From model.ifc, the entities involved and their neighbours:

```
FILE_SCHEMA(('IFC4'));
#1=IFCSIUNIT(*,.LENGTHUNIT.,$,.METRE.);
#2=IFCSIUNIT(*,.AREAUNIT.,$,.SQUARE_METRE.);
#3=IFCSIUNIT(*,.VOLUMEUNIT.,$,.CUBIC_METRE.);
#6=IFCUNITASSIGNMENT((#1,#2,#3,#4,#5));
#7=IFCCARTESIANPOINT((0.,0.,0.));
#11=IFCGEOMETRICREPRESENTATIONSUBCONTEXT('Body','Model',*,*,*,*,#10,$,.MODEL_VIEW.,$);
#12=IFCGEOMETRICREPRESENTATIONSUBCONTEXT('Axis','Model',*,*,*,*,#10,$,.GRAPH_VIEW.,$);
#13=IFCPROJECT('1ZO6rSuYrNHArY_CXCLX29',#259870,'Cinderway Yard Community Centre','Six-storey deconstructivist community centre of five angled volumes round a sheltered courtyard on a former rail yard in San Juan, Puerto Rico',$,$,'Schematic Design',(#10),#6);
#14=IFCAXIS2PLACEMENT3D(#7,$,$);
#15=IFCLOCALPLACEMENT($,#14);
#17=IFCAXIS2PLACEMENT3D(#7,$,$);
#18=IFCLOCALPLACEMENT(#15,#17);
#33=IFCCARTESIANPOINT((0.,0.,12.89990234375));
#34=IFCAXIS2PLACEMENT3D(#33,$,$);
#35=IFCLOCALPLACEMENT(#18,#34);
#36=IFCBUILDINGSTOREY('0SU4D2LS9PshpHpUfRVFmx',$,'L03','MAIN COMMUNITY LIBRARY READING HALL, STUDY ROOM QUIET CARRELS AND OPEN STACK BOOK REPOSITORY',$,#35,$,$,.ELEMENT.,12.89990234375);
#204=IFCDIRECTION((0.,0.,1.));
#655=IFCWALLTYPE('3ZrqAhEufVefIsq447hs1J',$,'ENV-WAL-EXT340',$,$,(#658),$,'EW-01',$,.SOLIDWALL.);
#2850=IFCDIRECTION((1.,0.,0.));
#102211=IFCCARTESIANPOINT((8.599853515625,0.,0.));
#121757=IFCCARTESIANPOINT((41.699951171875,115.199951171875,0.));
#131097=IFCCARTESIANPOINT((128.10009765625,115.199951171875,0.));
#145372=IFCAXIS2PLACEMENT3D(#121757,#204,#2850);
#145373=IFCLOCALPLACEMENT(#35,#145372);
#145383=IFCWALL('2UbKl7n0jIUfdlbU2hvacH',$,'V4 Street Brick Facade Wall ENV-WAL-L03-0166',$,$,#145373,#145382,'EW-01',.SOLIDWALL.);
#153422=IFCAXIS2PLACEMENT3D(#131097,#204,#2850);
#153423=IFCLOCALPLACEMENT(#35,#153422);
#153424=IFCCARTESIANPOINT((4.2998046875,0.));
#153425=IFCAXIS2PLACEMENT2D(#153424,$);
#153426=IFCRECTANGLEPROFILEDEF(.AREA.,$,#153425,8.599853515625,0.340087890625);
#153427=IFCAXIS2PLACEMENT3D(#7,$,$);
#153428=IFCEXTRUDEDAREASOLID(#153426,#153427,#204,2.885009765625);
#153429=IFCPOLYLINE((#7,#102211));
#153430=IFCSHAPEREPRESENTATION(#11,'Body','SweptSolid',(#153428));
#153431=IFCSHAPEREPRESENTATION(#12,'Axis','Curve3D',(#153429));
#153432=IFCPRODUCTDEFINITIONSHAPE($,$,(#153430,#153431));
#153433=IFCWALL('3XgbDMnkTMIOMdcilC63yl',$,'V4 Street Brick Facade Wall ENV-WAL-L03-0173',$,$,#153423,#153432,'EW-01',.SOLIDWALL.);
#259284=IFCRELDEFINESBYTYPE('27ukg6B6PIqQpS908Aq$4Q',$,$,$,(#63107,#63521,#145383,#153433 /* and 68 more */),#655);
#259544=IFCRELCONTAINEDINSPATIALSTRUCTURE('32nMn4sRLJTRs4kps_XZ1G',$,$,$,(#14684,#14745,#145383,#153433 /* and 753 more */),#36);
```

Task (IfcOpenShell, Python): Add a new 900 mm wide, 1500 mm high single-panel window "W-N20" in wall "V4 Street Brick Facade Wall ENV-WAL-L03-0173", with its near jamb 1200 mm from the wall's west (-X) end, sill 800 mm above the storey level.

```python
import numpy as np
import ifcopenshell
import ifcopenshell.api.feature
import ifcopenshell.api.geometry
import ifcopenshell.api.root
import ifcopenshell.api.spatial
import ifcopenshell.geom
import ifcopenshell.util.element
import ifcopenshell.util.placement
import ifcopenshell.util.representation
import ifcopenshell.util.shape
import ifcopenshell.util.unit

model = ifcopenshell.open("model.ifc")
unit_scale = ifcopenshell.util.unit.calculate_unit_scale(model)
settings = ifcopenshell.geom.settings()


def volume(element):
    """Net volume in cubic metres, openings subtracted."""
    shape = ifcopenshell.geom.create_shape(settings, element)
    return ifcopenshell.util.shape.get_volume(shape.geometry)


wall = model.by_guid("3XgbDMnkTMIOMdcilC63yl")
storey = ifcopenshell.util.element.get_container(wall, ifc_class="IfcBuildingStorey")
context = ifcopenshell.util.representation.get_context(model, "Model", "Body", "MODEL_VIEW")
before = volume(wall)

width, height, from_end, sill = 0.9, 1.5, 1.2, 0.8  # metres

# The wall runs along its own X axis, and the end named is its -X end.
wall_shape = ifcopenshell.geom.create_shape(settings, wall)
x, y, z = ifcopenshell.util.shape.get_vertices(wall_shape.geometry).T
start = x.min() + from_end
face, thickness = float(y.min()), float(y.max() - y.min())
wall_matrix = ifcopenshell.util.placement.get_local_placement(wall.ObjectPlacement)
level = ifcopenshell.util.placement.get_local_placement(storey.ObjectPlacement)[2, 3]


def in_wall(x, y):
    """Placement at x, y metres in the wall's axes, at sill height."""
    matrix = wall_matrix.copy()
    matrix[:, 3] = wall_matrix @ np.array([x / unit_scale, y / unit_scale, 0.0, 1.0])
    matrix[2, 3] = level + sill / unit_scale
    return matrix


# Opening: a box that overshoots both wall faces by 50 mm.
opening = ifcopenshell.api.root.create_entity(model, ifc_class="IfcOpeningElement", predefined_type="OPENING")
box = ifcopenshell.api.geometry.add_wall_representation(
    model, context=context, length=width, height=height, thickness=thickness + 0.1
)
ifcopenshell.api.geometry.assign_representation(model, product=opening, representation=box)
ifcopenshell.api.geometry.edit_object_placement(model, product=opening, matrix=in_wall(start, face - 0.05), is_si=False)
ifcopenshell.api.feature.add_feature(model, feature=opening, element=wall)

window = ifcopenshell.api.root.create_entity(model, ifc_class="IfcWindow", name="W-N20", predefined_type="WINDOW")
window.OverallWidth, window.OverallHeight = width / unit_scale, height / unit_scale
window.PartitioningType = "SINGLE_PANEL"
body = ifcopenshell.api.geometry.add_window_representation(
    model,
    context=context,
    overall_width=window.OverallWidth,
    overall_height=window.OverallHeight,
    partition_type="SINGLE_PANEL",
)
ifcopenshell.api.geometry.assign_representation(model, product=window, representation=body)
ifcopenshell.api.spatial.assign_container(model, products=[window], relating_structure=storey)
ifcopenshell.api.feature.add_filling(model, opening=opening, element=window)

# Centre the window in the wall's thickness.
ifcopenshell.api.geometry.edit_object_placement(model, product=window, matrix=in_wall(start, face), is_si=False)
window_shape = ifcopenshell.geom.create_shape(settings, window)
depth = ifcopenshell.util.shape.get_vertices(window_shape.geometry)[:, 1]
offset = face + thickness / 2 - (depth.min() + depth.max()) / 2
ifcopenshell.api.geometry.edit_object_placement(model, product=window, matrix=in_wall(start, offset), is_si=False)

after = volume(wall)

print(f"wall volume {before:.3f} -> {after:.3f} m3")

model.write("model_edited.ifc")
```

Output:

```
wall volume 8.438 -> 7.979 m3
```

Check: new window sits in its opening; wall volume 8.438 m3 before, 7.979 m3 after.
